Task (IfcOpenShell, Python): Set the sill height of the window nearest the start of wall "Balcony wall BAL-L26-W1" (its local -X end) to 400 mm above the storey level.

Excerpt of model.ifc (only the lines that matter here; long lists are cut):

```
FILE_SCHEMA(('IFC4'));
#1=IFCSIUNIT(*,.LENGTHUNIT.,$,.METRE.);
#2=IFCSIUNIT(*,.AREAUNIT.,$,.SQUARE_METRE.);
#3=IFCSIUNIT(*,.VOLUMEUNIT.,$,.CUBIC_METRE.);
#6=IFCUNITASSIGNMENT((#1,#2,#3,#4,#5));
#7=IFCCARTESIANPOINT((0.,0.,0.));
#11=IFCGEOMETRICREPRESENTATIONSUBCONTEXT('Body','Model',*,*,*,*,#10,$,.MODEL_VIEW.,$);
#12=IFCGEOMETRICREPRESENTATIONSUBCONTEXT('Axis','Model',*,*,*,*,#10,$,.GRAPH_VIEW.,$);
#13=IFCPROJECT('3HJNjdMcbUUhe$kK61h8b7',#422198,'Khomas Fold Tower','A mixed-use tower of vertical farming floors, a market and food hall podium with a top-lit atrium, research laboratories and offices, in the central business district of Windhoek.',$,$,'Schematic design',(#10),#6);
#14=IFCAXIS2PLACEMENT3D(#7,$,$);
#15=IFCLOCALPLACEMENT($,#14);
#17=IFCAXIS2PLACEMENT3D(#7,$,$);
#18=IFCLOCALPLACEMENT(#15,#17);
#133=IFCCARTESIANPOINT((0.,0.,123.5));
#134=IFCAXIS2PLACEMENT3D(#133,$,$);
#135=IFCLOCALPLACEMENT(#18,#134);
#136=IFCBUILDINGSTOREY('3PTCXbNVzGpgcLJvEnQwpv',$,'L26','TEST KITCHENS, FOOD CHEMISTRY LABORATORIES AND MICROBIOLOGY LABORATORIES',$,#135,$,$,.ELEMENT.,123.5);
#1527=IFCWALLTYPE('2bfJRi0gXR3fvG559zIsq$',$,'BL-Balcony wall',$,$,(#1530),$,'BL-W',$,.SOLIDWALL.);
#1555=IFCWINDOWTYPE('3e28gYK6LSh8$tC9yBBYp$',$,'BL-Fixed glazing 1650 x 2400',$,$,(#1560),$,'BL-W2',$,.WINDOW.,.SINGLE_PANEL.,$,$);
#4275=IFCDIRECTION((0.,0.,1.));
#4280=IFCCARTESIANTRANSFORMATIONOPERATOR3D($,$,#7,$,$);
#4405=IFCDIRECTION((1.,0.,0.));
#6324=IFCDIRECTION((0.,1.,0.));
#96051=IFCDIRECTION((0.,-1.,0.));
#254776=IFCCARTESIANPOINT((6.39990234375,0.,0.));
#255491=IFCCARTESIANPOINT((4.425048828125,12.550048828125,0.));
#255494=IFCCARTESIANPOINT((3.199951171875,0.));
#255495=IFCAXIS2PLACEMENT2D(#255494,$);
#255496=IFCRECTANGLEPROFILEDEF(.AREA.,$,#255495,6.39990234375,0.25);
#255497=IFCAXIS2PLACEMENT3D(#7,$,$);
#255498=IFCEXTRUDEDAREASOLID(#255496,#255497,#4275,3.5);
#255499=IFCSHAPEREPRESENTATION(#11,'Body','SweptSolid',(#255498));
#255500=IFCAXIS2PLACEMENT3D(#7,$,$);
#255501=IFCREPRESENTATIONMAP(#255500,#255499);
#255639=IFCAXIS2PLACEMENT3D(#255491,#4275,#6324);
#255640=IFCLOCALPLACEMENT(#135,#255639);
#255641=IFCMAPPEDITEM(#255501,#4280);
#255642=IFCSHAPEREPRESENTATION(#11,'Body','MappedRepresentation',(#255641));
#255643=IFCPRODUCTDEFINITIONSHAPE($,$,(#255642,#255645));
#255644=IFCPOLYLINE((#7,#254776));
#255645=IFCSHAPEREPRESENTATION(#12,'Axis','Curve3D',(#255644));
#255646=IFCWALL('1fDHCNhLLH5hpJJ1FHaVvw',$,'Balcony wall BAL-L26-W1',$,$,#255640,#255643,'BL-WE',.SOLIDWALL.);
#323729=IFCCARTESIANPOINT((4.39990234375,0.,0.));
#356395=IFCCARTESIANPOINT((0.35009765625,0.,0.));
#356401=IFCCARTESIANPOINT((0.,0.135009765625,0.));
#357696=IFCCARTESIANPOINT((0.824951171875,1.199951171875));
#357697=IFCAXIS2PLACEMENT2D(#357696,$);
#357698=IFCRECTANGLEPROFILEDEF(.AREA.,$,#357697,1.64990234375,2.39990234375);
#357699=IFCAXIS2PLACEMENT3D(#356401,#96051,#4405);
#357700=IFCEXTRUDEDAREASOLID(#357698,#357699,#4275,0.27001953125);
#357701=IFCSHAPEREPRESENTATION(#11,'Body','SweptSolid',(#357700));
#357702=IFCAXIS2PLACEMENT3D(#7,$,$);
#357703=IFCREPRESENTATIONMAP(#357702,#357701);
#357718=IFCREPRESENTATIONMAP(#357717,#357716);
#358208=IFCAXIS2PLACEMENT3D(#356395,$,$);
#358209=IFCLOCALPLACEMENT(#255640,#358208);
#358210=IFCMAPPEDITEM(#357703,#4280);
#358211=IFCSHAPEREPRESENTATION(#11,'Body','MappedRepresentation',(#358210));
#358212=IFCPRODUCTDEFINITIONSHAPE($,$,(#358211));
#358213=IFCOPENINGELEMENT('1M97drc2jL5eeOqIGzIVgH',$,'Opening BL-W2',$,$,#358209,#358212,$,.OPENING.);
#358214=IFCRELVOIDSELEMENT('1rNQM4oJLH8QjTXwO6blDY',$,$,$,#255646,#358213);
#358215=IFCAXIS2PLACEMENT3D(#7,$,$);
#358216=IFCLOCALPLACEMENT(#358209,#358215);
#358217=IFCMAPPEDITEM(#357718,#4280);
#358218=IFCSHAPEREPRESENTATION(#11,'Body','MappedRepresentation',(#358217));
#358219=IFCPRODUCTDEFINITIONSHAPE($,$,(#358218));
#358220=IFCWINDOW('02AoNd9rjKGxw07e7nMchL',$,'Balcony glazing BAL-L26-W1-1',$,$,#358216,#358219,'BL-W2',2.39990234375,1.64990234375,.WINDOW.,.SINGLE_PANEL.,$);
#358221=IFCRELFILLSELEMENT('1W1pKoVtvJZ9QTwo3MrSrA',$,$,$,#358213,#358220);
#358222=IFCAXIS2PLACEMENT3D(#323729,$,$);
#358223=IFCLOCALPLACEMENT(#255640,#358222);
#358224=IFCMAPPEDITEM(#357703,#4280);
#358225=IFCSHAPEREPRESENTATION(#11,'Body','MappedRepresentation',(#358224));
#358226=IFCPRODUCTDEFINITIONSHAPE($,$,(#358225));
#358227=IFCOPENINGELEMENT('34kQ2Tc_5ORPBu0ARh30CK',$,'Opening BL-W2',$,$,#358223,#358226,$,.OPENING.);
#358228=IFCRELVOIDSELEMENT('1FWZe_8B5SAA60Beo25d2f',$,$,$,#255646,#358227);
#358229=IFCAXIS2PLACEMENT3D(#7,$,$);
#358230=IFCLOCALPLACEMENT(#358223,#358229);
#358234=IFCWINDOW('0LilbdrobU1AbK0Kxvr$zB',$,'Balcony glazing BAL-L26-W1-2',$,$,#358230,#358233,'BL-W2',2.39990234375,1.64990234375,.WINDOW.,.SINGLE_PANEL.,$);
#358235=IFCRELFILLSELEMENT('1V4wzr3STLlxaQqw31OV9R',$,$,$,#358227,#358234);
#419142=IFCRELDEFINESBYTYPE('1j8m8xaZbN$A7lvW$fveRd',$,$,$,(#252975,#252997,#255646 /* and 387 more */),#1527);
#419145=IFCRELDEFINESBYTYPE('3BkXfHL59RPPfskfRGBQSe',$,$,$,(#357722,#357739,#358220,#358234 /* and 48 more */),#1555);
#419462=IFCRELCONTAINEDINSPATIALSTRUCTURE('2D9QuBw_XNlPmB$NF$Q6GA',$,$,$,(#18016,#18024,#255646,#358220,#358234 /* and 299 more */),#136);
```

```python
import numpy as np
import ifcopenshell
import ifcopenshell.api.geometry
import ifcopenshell.geom
import ifcopenshell.util.element
import ifcopenshell.util.placement
import ifcopenshell.util.shape
import ifcopenshell.util.unit

model = ifcopenshell.open("model.ifc")
unit_scale = ifcopenshell.util.unit.calculate_unit_scale(model)

window = model.by_id(358220)
opening = window.FillsVoids[0].RelatingOpeningElement
storey = ifcopenshell.util.element.get_container(window, ifc_class="IfcBuildingStorey")
level = ifcopenshell.util.placement.get_local_placement(storey.ObjectPlacement)[2, 3]

# The opening's origin need not be at the sill, so measure its lowest point.
shape = ifcopenshell.geom.create_shape(ifcopenshell.geom.settings(), opening)
bottom = ifcopenshell.util.shape.get_shape_bottom_elevation(shape, shape.geometry) / unit_scale
dz = level + 0.4 - bottom

shift = np.array([0.0, 0.0, dz])
# The window is placed relative to its opening, so it follows when the opening moves.
matrix = ifcopenshell.util.placement.get_local_placement(opening.ObjectPlacement)
matrix[:3, 3] += shift
ifcopenshell.api.geometry.edit_object_placement(
    model, product=opening, matrix=matrix, is_si=False, should_transform_children=True
)

print(f"moved by {dz * unit_scale:+.3f} m")

model.write("model_rev.ifc")
```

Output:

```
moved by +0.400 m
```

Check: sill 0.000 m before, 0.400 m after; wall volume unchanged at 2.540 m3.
